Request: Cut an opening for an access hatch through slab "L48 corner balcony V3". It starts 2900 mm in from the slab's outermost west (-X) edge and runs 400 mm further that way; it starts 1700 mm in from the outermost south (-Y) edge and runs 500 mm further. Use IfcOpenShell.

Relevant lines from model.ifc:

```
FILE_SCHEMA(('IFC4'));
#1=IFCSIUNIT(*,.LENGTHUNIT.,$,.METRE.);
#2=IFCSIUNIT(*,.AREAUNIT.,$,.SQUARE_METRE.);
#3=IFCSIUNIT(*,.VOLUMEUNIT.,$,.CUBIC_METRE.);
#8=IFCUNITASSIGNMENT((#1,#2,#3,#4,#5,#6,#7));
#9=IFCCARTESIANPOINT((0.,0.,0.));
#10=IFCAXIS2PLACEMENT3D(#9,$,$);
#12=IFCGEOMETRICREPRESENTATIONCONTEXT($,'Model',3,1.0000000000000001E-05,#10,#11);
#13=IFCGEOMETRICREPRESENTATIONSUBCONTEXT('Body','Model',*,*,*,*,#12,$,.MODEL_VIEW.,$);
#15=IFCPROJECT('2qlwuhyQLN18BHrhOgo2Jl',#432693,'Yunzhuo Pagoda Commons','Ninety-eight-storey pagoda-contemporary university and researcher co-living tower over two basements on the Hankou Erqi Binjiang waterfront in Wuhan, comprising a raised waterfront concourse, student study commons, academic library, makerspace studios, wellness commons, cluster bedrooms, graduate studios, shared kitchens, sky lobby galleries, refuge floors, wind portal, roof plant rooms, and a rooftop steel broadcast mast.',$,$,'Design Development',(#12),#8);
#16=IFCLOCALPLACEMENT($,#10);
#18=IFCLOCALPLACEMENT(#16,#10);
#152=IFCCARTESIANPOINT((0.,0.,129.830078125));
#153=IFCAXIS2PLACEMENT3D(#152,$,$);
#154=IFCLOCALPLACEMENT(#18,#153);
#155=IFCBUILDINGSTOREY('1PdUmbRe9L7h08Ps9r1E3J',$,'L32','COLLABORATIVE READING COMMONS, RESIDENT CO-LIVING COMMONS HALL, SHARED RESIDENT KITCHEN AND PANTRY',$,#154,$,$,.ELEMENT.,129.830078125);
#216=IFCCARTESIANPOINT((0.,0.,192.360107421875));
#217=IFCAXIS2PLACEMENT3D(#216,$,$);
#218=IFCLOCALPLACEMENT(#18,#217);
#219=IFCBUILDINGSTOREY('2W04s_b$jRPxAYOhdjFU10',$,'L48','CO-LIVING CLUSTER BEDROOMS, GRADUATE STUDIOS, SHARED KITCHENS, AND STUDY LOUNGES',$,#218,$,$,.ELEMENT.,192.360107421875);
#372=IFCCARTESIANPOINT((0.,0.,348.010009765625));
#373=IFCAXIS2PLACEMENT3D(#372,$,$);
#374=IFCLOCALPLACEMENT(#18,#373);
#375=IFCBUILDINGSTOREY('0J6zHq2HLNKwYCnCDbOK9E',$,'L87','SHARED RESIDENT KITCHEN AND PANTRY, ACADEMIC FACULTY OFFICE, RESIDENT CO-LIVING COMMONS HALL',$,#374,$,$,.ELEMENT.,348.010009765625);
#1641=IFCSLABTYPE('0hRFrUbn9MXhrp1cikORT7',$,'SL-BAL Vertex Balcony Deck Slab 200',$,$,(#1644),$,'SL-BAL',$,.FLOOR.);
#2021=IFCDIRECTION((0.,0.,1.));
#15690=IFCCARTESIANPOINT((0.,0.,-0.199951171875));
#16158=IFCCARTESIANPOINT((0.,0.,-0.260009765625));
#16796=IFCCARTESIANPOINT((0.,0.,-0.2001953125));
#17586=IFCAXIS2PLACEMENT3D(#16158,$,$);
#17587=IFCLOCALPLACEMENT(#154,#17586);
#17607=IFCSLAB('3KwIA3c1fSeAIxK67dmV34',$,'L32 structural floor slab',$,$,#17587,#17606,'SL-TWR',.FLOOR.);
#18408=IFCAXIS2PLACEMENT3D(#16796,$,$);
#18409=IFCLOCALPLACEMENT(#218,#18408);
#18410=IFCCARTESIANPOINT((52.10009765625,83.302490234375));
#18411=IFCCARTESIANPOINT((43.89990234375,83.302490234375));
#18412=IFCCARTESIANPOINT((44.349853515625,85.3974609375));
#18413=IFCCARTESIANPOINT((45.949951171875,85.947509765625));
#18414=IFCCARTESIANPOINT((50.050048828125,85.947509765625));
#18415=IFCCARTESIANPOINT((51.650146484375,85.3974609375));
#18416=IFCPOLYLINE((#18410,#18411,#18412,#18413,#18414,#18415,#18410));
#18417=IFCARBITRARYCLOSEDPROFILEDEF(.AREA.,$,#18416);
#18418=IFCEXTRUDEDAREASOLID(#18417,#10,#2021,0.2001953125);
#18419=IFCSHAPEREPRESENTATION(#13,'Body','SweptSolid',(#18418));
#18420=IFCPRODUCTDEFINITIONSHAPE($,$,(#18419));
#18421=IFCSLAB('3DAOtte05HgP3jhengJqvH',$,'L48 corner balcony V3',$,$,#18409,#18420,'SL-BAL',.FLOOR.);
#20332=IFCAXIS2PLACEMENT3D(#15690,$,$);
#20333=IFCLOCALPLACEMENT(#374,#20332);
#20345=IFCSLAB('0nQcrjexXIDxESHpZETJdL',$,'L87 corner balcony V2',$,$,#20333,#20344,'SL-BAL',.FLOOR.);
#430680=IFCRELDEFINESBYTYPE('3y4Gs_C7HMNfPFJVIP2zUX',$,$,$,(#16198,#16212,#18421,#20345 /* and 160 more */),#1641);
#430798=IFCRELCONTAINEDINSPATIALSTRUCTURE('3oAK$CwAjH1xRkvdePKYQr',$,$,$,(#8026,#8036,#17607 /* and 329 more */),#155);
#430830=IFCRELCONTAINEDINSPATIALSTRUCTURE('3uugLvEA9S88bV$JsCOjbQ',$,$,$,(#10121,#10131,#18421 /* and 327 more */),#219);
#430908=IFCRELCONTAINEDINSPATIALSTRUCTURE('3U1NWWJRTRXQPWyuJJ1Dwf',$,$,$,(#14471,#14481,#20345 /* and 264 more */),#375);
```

```python
import numpy as np
import ifcopenshell
import ifcopenshell.api.feature
import ifcopenshell.api.geometry
import ifcopenshell.api.root
import ifcopenshell.geom
import ifcopenshell.util.placement
import ifcopenshell.util.representation
import ifcopenshell.util.shape
import ifcopenshell.util.unit

model = ifcopenshell.open("model.ifc")
unit_scale = ifcopenshell.util.unit.calculate_unit_scale(model)
settings = ifcopenshell.geom.settings()


def volume(element):
    """Net volume in cubic metres, openings subtracted."""
    shape = ifcopenshell.geom.create_shape(settings, element)
    return ifcopenshell.util.shape.get_volume(shape.geometry)


slab = model.by_guid("3DAOtte05HgP3jhengJqvH")
before = volume(slab)

# Extent in the slab's own axes, in metres. The edges named are its -X and -Y sides.
slab_shape = ifcopenshell.geom.create_shape(settings, slab)
vertices = ifcopenshell.util.shape.get_vertices(slab_shape.geometry)
x_min, y_min, bottom = vertices.min(axis=0)
top = vertices[:, 2].max()

opening = ifcopenshell.api.root.create_entity(model, ifc_class="IfcOpeningElement", name="Access hatch opening", predefined_type="OPENING")
context = ifcopenshell.util.representation.get_context(model, "Model", "Body", "MODEL_VIEW")
width, depth = 0.4, 0.5
outline = [(0.0, 0.0), (width, 0.0), (width, depth), (0.0, depth), (0.0, 0.0)]
# Overshoot both faces by 50 mm so the cut is clean.
shape = ifcopenshell.api.geometry.add_slab_representation(
    model, context=context, depth=top - bottom + 0.1, polyline=outline
)
ifcopenshell.api.geometry.assign_representation(model, product=opening, representation=shape)

matrix = ifcopenshell.util.placement.get_local_placement(slab.ObjectPlacement)
matrix[:, 3] = matrix @ np.append(np.array([x_min + 2.9, y_min + 1.7, bottom - 0.05]) / unit_scale, 1.0)
ifcopenshell.api.geometry.edit_object_placement(model, product=opening, matrix=matrix, is_si=False)
ifcopenshell.api.feature.add_feature(model, feature=opening, element=slab)

after = volume(slab)

print(f"slab volume {before:.3f} -> {after:.3f} m3")

model.write("model_updated.ifc")
```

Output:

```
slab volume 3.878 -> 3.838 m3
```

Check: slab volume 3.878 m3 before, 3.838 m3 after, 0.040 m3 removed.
